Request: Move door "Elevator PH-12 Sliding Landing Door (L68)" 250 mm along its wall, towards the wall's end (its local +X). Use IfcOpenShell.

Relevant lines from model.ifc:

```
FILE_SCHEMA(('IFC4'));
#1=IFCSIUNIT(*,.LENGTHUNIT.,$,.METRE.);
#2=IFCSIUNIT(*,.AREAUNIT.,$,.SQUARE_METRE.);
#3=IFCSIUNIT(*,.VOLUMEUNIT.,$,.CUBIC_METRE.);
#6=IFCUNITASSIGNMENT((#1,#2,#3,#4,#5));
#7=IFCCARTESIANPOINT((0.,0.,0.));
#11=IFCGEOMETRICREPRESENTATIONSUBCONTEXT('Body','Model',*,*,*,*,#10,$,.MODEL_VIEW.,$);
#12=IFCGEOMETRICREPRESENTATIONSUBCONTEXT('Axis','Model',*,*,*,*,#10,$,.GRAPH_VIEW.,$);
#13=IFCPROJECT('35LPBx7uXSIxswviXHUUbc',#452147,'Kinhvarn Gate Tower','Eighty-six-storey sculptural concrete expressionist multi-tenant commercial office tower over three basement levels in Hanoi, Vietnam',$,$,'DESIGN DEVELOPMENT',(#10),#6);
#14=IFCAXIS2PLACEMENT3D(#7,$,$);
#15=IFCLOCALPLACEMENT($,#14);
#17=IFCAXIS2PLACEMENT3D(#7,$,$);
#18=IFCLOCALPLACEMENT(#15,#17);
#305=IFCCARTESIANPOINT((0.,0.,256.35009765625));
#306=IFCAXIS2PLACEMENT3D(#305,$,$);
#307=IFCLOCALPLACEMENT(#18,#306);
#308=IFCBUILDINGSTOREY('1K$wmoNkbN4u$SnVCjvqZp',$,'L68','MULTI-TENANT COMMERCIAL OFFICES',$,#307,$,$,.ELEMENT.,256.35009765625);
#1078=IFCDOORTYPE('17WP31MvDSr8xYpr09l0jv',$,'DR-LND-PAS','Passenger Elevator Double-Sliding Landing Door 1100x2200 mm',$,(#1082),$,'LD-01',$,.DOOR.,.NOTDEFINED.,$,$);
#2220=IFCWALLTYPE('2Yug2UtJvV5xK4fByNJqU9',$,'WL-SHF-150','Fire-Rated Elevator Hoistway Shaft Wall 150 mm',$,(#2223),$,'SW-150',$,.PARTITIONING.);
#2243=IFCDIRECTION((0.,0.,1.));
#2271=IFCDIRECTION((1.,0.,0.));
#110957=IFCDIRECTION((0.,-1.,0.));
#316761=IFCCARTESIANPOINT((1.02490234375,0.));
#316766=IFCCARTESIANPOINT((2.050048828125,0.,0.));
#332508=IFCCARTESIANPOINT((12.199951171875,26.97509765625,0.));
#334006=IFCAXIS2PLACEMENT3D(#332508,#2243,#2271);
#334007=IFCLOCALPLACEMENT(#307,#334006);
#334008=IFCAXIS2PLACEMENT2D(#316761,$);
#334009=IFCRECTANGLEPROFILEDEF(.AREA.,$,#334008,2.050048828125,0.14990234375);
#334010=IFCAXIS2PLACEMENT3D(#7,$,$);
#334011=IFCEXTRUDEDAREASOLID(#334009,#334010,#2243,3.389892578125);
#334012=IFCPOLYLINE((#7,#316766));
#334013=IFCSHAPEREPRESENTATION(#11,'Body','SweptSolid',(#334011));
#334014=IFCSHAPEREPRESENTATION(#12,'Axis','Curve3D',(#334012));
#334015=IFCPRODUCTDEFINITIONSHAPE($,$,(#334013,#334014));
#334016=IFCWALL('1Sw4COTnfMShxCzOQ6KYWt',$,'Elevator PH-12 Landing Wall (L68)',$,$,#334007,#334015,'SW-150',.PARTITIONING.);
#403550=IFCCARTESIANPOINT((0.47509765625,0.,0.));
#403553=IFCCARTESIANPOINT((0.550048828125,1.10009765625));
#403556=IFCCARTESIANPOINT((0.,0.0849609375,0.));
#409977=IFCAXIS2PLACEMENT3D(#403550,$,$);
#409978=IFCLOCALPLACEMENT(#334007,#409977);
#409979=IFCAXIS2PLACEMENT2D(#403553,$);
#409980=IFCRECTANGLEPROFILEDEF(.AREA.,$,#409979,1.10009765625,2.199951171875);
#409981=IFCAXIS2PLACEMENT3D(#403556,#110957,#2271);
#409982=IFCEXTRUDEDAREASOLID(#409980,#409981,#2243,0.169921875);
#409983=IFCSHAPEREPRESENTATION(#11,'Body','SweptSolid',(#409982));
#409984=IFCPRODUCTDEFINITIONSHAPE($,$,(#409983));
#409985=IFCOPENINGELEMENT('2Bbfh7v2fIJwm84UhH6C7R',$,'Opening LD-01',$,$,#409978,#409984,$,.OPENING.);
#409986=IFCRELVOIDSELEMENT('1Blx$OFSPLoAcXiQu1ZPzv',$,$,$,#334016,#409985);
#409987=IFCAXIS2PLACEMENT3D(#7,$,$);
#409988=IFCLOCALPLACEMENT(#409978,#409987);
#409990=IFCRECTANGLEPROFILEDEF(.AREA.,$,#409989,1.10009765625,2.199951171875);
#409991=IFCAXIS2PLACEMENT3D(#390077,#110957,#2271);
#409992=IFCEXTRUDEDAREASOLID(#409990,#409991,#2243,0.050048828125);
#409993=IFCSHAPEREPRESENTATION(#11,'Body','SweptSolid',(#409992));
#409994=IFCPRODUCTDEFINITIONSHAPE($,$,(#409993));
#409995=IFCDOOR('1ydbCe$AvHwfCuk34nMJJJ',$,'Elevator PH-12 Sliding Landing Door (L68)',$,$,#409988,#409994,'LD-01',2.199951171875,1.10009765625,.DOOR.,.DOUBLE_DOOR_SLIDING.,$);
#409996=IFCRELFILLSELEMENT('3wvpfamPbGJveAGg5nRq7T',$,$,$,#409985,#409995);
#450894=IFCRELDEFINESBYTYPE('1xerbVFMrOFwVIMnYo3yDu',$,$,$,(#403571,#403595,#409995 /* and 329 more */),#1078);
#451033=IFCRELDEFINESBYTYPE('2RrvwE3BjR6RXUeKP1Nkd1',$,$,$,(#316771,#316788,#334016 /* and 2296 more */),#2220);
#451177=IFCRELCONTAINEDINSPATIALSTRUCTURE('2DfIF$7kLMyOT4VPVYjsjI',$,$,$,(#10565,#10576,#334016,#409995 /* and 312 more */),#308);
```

```python
import ifcopenshell
import ifcopenshell.api.geometry
import ifcopenshell.util.placement

model = ifcopenshell.open("model.ifc")

door = model.by_id(409995)
opening = door.FillsVoids[0].RelatingOpeningElement
wall = opening.VoidsElements[0].RelatingBuildingElement

wall_matrix = ifcopenshell.util.placement.get_local_placement(wall.ObjectPlacement)
shift = wall_matrix[:3, 0] * 0.25
before = ifcopenshell.util.placement.get_local_placement(door.ObjectPlacement)[:3, 3].copy()

# The door is placed relative to its opening, so it follows when the opening moves.
matrix = ifcopenshell.util.placement.get_local_placement(opening.ObjectPlacement)
matrix[:3, 3] += shift
ifcopenshell.api.geometry.edit_object_placement(
    model, product=opening, matrix=matrix, is_si=False, should_transform_children=True
)

after = ifcopenshell.util.placement.get_local_placement(door.ObjectPlacement)[:3, 3]
print("door moved by", (after - before).round(3) + 0.0)

model.write("model_updated.ifc")
```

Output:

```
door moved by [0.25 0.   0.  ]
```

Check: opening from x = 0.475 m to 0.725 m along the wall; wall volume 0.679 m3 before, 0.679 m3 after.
